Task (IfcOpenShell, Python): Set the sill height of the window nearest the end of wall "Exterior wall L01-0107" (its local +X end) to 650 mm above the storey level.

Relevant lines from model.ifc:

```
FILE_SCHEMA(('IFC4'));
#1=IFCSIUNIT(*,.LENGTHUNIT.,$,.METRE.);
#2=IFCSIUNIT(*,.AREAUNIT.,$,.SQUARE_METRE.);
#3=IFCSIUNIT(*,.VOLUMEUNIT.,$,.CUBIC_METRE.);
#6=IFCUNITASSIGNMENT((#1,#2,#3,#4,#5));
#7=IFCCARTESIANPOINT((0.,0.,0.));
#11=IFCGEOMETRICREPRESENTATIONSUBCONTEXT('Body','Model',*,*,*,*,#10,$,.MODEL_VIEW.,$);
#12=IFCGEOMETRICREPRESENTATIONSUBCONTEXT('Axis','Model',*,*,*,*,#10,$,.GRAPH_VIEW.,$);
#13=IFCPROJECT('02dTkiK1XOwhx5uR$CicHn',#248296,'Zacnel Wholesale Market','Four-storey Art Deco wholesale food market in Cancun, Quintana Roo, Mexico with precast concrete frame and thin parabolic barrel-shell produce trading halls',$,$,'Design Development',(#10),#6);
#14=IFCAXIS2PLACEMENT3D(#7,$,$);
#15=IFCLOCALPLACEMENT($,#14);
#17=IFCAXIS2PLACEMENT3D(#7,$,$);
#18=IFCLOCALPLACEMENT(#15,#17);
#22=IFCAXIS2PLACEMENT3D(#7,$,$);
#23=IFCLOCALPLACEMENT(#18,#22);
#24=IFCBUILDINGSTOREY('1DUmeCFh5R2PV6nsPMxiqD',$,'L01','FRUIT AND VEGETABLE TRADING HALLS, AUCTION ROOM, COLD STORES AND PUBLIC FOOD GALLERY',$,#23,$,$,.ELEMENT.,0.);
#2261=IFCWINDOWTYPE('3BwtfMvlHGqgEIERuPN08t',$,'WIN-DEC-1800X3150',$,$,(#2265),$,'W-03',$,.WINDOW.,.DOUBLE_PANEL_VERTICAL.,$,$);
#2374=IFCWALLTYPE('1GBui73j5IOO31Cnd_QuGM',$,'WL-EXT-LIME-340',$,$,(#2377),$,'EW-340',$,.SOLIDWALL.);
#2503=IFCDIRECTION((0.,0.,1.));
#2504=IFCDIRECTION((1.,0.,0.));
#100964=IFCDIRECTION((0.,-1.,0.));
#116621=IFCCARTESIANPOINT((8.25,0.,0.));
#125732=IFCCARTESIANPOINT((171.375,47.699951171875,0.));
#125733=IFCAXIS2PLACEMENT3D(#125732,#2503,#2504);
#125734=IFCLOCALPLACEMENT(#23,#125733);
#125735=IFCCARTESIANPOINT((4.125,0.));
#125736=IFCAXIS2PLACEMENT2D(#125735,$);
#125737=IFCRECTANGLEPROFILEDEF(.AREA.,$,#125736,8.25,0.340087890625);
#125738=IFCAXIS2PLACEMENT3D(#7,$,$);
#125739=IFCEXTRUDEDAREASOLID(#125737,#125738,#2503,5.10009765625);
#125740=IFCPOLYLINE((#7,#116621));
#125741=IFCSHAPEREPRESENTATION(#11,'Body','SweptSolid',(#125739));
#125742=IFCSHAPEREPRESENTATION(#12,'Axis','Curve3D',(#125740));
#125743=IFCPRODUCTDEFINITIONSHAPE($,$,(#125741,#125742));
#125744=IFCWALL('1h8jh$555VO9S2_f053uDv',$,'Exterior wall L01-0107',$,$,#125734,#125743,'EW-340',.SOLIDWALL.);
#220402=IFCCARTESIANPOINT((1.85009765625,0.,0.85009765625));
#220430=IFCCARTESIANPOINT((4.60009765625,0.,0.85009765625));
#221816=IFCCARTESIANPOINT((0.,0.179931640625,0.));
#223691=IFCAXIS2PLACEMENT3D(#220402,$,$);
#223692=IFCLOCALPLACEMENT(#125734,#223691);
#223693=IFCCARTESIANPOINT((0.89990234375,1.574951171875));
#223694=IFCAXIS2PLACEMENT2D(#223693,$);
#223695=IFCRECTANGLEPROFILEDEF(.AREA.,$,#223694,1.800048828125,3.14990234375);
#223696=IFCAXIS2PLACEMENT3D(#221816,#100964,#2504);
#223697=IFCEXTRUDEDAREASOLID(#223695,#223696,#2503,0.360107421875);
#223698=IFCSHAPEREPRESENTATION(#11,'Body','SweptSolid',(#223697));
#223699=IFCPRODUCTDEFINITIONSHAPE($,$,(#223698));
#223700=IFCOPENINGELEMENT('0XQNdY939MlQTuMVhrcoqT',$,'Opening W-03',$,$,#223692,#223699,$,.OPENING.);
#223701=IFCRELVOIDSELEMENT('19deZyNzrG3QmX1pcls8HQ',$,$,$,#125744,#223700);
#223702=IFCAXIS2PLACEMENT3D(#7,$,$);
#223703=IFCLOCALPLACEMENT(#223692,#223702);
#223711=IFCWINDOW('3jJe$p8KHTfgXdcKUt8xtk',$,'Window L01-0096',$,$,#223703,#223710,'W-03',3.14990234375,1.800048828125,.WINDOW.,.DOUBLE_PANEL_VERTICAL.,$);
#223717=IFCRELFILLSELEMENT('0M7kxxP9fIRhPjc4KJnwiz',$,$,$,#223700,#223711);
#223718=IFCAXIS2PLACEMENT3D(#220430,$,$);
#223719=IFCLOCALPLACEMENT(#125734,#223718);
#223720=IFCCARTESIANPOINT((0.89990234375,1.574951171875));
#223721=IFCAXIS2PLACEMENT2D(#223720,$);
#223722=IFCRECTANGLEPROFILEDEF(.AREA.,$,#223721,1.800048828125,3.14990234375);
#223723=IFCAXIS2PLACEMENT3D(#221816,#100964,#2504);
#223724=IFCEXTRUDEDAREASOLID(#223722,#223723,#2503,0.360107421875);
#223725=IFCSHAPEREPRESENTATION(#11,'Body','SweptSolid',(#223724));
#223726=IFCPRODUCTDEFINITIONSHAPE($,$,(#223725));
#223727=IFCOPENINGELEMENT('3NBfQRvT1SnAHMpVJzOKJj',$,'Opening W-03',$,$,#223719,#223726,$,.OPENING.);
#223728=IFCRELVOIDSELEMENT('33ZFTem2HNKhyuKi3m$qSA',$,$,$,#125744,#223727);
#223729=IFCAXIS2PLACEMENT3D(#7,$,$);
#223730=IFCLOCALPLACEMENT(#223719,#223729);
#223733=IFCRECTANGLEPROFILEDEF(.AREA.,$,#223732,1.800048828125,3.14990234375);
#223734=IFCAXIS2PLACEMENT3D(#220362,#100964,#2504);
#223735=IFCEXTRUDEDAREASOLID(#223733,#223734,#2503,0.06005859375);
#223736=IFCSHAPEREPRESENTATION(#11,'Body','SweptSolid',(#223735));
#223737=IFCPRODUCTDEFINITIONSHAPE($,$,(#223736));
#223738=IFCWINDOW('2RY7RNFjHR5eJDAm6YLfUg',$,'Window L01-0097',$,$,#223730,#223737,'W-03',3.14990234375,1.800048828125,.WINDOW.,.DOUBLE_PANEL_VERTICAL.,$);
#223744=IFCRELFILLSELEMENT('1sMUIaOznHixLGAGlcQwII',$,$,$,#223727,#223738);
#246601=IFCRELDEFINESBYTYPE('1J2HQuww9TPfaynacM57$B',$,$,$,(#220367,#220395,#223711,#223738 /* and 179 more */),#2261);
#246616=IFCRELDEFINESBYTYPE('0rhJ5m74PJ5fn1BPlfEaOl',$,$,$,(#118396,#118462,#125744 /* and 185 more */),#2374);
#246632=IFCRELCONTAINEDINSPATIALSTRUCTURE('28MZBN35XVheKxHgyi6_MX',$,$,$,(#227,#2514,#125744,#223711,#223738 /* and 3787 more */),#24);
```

```python
import numpy as np
import ifcopenshell
import ifcopenshell.api.geometry
import ifcopenshell.geom
import ifcopenshell.util.element
import ifcopenshell.util.placement
import ifcopenshell.util.shape
import ifcopenshell.util.unit

model = ifcopenshell.open("model.ifc")
unit_scale = ifcopenshell.util.unit.calculate_unit_scale(model)

window = model.by_guid("2RY7RNFjHR5eJDAm6YLfUg")
opening = window.FillsVoids[0].RelatingOpeningElement
storey = ifcopenshell.util.element.get_container(window, ifc_class="IfcBuildingStorey")
level = ifcopenshell.util.placement.get_local_placement(storey.ObjectPlacement)[2, 3]

# The opening's origin need not be at the sill, so measure its lowest point.
shape = ifcopenshell.geom.create_shape(ifcopenshell.geom.settings(), opening)
bottom = ifcopenshell.util.shape.get_shape_bottom_elevation(shape, shape.geometry) / unit_scale
dz = level + 0.65 / unit_scale - bottom

shift = np.array([0.0, 0.0, dz])
# The window is placed relative to its opening, so it follows when the opening moves.
matrix = ifcopenshell.util.placement.get_local_placement(opening.ObjectPlacement)
matrix[:3, 3] += shift
ifcopenshell.api.geometry.edit_object_placement(
    model, product=opening, matrix=matrix, is_si=False, should_transform_children=True
)

print(f"moved by {dz * unit_scale:+.3f} m")

model.write("model-out.ifc")
```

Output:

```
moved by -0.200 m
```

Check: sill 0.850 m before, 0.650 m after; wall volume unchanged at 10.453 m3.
